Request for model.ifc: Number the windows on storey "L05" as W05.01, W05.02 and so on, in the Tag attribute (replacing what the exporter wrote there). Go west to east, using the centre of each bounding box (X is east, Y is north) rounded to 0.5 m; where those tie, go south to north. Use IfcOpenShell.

First a look at what the model holds.

```python
import ifcopenshell
import ifcopenshell.util.element
import ifcopenshell.util.placement

model = ifcopenshell.open("model.ifc")
print(model.schema)
storey = next(s for s in model.by_type("IfcBuildingStorey") if s.Name == "L05")
windows = [e for e in ifcopenshell.util.element.get_decomposition(storey) if e.is_a("IfcWindow")]
for e in sorted(windows, key=lambda e: e.id()):
    origin = ifcopenshell.util.placement.get_local_placement(e.ObjectPlacement)[:3, 3]
    print(e.id(), e.Tag, e.Name, origin.round(2) + 0.0, sep=" | ")
```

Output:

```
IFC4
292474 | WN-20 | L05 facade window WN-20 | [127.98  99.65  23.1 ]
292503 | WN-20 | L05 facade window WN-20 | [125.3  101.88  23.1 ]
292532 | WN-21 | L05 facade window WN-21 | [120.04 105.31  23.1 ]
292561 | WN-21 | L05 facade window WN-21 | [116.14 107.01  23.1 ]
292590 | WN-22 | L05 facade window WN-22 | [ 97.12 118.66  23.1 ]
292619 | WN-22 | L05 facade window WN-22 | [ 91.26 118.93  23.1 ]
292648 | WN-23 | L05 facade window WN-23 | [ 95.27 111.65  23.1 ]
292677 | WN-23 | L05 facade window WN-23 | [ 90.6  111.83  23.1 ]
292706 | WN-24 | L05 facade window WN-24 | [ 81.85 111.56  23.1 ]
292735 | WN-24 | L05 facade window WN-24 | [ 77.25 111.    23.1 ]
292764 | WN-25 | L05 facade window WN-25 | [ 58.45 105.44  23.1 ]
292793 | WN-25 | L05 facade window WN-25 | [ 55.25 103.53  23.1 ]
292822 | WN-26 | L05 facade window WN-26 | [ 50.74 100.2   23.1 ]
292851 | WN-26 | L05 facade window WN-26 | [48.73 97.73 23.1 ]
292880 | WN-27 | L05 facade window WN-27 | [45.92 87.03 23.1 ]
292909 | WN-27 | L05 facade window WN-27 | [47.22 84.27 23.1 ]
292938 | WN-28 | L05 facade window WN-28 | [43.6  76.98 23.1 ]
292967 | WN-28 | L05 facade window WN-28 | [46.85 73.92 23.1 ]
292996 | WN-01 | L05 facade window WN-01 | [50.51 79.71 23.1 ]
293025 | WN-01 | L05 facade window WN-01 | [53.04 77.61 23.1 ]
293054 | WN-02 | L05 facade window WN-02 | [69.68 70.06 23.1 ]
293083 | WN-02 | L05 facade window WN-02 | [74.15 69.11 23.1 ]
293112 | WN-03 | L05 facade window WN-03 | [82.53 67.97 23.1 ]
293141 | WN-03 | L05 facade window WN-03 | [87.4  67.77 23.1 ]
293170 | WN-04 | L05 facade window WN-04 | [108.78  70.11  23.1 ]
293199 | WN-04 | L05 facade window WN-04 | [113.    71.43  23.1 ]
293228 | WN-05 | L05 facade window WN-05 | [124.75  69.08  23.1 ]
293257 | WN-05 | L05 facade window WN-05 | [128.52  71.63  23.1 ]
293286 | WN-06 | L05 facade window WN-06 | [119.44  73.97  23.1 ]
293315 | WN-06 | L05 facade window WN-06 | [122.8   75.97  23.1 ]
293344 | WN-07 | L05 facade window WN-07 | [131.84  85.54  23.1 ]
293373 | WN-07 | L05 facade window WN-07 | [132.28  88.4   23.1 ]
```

```python
import ifcopenshell
import ifcopenshell.geom
import ifcopenshell.util.element
import ifcopenshell.util.shape

model = ifcopenshell.open("model.ifc")
settings = ifcopenshell.geom.settings()
settings.set("use-world-coords", True)


def centre(element):
    shape = ifcopenshell.geom.create_shape(settings, element)
    return ifcopenshell.util.shape.get_bbox_centroid(shape.geometry)


storey = next(s for s in model.by_type("IfcBuildingStorey") if s.Name == "L05")
windows = [e for e in ifcopenshell.util.element.get_decomposition(storey) if e.is_a("IfcWindow")]

# Insertion points can sit at a corner or the storey origin, so sort by the geometry (in metres).
centres = {e: centre(e) for e in windows}
windows.sort(key=lambda e: (round(centres[e][0] / 0.5), centres[e][1]))

for i, e in enumerate(windows, start=1):
    number = f"W05.{i:02d}"
    e.Tag = number
    print(e.id(), number)

model.write("model_v2.ifc")
```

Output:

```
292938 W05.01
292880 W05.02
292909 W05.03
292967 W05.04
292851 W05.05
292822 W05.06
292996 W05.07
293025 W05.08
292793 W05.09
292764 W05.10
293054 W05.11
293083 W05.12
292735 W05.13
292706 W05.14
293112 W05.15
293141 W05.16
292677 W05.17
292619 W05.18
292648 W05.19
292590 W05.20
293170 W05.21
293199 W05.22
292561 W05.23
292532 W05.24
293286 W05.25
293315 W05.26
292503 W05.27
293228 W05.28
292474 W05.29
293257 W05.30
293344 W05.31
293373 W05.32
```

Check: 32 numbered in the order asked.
